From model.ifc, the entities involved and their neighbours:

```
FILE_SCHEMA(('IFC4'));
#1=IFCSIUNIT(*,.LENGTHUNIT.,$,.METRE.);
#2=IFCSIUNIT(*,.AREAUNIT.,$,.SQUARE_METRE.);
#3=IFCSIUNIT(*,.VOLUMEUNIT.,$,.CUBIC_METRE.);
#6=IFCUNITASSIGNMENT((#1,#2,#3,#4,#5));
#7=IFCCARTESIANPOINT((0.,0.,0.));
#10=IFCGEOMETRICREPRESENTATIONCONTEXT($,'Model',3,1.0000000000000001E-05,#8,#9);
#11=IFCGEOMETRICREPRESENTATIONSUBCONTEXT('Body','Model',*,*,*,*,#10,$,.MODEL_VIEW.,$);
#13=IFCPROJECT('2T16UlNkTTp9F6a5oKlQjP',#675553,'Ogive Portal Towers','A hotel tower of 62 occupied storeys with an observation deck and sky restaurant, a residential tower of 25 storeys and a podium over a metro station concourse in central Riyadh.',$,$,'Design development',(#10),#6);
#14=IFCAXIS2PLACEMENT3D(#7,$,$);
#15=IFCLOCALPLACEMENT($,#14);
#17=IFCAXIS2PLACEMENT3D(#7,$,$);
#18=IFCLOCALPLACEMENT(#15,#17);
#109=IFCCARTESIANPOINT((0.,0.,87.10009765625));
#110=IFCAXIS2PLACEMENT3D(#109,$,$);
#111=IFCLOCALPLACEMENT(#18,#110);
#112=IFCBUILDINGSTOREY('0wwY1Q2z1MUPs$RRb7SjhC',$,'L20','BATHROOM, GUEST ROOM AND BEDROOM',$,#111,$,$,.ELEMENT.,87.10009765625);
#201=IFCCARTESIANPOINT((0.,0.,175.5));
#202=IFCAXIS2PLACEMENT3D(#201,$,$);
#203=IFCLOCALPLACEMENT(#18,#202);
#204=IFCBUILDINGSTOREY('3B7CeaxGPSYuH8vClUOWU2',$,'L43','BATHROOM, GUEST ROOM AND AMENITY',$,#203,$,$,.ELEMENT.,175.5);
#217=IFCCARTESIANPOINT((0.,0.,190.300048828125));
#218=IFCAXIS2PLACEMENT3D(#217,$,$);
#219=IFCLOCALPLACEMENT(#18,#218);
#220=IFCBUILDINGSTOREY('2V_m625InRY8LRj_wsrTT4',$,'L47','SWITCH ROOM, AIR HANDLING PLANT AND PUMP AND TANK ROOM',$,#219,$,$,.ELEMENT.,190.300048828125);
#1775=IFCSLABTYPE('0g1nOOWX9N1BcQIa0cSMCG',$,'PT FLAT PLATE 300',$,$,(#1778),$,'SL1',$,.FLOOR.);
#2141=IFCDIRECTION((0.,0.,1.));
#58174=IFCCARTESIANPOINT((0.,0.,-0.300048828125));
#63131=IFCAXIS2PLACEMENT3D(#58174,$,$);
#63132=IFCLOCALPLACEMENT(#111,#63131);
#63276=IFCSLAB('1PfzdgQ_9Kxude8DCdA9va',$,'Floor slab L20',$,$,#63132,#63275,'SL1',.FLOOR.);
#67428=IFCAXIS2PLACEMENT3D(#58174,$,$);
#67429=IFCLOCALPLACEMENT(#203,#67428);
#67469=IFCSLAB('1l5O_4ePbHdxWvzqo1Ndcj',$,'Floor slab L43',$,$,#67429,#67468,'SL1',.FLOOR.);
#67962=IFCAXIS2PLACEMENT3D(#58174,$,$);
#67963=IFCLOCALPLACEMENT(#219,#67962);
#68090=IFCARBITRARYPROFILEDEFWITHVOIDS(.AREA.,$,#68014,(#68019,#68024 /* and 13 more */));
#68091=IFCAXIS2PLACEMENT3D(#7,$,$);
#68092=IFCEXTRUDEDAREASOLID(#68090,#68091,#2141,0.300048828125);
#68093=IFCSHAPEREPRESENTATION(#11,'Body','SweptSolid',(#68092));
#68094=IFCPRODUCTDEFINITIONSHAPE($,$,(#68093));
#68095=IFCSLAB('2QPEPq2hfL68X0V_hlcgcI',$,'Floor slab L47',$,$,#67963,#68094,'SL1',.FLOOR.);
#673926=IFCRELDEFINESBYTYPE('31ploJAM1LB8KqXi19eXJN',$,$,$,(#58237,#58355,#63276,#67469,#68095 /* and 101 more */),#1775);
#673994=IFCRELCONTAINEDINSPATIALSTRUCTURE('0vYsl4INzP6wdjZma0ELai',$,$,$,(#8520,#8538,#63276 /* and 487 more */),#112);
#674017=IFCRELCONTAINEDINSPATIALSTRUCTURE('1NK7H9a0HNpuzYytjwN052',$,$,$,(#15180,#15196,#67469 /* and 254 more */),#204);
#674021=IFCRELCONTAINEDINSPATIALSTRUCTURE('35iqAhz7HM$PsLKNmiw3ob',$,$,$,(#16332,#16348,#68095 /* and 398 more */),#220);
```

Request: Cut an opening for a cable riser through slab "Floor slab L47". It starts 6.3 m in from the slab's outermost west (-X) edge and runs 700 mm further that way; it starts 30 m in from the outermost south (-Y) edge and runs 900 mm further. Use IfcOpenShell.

```python
import numpy as np
import ifcopenshell
import ifcopenshell.api.feature
import ifcopenshell.api.geometry
import ifcopenshell.api.root
import ifcopenshell.geom
import ifcopenshell.util.placement
import ifcopenshell.util.representation
import ifcopenshell.util.shape
import ifcopenshell.util.unit

model = ifcopenshell.open("model.ifc")
unit_scale = ifcopenshell.util.unit.calculate_unit_scale(model)
settings = ifcopenshell.geom.settings()


def volume(element):
    """Net volume in cubic metres, openings subtracted."""
    shape = ifcopenshell.geom.create_shape(settings, element)
    return ifcopenshell.util.shape.get_volume(shape.geometry)


slab = model.by_guid("2QPEPq2hfL68X0V_hlcgcI")
before = volume(slab)

# Extent in the slab's own axes, in metres. The edges named are its -X and -Y sides.
slab_shape = ifcopenshell.geom.create_shape(settings, slab)
vertices = ifcopenshell.util.shape.get_vertices(slab_shape.geometry)
x_min, y_min, bottom = vertices.min(axis=0)
top = vertices[:, 2].max()

opening = ifcopenshell.api.root.create_entity(model, ifc_class="IfcOpeningElement", name="Cable riser opening", predefined_type="OPENING")
context = ifcopenshell.util.representation.get_context(model, "Model", "Body", "MODEL_VIEW")
width, depth = 0.7, 0.9
outline = [(0.0, 0.0), (width, 0.0), (width, depth), (0.0, depth), (0.0, 0.0)]
# Overshoot both faces by 50 mm so the cut is clean.
shape = ifcopenshell.api.geometry.add_slab_representation(
    model, context=context, depth=top - bottom + 0.1, polyline=outline
)
ifcopenshell.api.geometry.assign_representation(model, product=opening, representation=shape)

matrix = ifcopenshell.util.placement.get_local_placement(slab.ObjectPlacement)
matrix[:, 3] = matrix @ np.append(np.array([x_min + 6.3, y_min + 30, bottom - 0.05]) / unit_scale, 1.0)
ifcopenshell.api.geometry.edit_object_placement(model, product=opening, matrix=matrix, is_si=False)
ifcopenshell.api.feature.add_feature(model, feature=opening, element=slab)

after = volume(slab)

print(f"slab volume {before:.3f} -> {after:.3f} m3")

model.write("model_edited.ifc")
```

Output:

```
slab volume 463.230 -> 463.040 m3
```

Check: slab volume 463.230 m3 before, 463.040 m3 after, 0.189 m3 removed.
